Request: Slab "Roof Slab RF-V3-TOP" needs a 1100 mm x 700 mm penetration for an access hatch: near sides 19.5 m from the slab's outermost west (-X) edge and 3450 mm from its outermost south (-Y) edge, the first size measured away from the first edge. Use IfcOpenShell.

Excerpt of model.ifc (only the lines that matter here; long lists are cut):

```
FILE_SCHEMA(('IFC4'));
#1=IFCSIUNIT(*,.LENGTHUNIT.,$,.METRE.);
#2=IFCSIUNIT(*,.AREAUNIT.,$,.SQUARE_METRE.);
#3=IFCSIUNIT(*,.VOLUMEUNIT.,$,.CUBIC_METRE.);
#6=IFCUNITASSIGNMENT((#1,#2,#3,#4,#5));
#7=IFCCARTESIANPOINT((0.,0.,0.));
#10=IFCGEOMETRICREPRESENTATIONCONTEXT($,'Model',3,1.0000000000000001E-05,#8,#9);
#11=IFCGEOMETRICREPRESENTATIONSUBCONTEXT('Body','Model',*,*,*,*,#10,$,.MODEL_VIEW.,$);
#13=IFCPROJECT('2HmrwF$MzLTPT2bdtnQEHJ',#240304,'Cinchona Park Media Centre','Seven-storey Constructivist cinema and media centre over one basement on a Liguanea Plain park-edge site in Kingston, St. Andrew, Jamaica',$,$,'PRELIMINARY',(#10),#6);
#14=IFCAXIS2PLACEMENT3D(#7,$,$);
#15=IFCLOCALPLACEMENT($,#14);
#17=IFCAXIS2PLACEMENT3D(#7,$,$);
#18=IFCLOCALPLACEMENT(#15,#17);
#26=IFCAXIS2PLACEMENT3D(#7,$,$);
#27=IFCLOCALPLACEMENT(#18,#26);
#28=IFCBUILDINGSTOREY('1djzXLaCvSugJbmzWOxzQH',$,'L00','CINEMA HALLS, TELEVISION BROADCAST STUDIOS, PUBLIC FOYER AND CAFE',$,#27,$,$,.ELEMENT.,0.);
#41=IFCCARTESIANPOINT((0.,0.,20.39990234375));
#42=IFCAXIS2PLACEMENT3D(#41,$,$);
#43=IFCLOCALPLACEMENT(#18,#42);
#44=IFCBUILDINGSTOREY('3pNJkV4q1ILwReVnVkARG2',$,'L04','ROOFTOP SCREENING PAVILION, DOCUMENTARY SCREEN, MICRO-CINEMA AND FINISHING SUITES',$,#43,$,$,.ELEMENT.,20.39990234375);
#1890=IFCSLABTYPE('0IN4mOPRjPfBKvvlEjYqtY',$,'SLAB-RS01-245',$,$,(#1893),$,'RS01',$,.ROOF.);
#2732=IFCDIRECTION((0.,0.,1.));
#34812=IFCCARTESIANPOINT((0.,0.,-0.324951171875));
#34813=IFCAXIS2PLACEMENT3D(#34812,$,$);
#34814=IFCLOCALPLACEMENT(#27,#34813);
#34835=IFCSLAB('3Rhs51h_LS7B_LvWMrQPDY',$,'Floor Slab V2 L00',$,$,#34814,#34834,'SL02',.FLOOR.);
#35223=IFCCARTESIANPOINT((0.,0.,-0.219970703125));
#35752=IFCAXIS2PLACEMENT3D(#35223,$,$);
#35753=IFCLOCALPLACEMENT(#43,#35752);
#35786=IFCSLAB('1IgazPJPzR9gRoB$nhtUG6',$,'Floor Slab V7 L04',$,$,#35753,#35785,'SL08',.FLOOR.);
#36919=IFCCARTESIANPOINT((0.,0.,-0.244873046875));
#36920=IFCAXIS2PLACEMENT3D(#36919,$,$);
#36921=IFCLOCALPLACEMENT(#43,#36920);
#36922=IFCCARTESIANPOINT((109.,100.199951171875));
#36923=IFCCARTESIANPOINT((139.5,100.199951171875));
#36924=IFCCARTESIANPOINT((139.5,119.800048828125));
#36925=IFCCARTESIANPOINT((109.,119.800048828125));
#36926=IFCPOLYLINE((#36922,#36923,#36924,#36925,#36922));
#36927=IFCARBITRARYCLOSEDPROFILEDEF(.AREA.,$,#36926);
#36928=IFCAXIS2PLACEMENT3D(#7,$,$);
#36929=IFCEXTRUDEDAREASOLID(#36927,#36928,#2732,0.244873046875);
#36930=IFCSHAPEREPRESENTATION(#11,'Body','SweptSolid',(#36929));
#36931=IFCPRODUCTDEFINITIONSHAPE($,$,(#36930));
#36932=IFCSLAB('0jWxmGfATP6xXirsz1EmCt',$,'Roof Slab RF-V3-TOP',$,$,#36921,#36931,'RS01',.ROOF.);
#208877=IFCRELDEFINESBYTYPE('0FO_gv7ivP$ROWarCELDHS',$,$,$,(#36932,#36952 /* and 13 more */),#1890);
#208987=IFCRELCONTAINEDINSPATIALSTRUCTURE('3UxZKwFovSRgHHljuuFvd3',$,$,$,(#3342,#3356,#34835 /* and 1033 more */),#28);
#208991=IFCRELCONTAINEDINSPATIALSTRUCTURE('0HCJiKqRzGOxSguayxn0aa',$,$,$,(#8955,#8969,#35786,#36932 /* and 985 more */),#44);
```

```python
import numpy as np
import ifcopenshell
import ifcopenshell.api.feature
import ifcopenshell.api.geometry
import ifcopenshell.api.root
import ifcopenshell.geom
import ifcopenshell.util.placement
import ifcopenshell.util.representation
import ifcopenshell.util.shape
import ifcopenshell.util.unit

model = ifcopenshell.open("model.ifc")
unit_scale = ifcopenshell.util.unit.calculate_unit_scale(model)
settings = ifcopenshell.geom.settings()


def volume(element):
    """Net volume in cubic metres, openings subtracted."""
    shape = ifcopenshell.geom.create_shape(settings, element)
    return ifcopenshell.util.shape.get_volume(shape.geometry)


slab = model.by_guid("0jWxmGfATP6xXirsz1EmCt")
before = volume(slab)

# Extent in the slab's own axes, in metres. The edges named are its -X and -Y sides.
slab_shape = ifcopenshell.geom.create_shape(settings, slab)
vertices = ifcopenshell.util.shape.get_vertices(slab_shape.geometry)
x_min, y_min, bottom = vertices.min(axis=0)
top = vertices[:, 2].max()

opening = ifcopenshell.api.root.create_entity(model, ifc_class="IfcOpeningElement", name="Access hatch opening", predefined_type="OPENING")
context = ifcopenshell.util.representation.get_context(model, "Model", "Body", "MODEL_VIEW")
width, depth = 1.1, 0.7
outline = [(0.0, 0.0), (width, 0.0), (width, depth), (0.0, depth), (0.0, 0.0)]
# Overshoot both faces by 50 mm so the cut is clean.
shape = ifcopenshell.api.geometry.add_slab_representation(
    model, context=context, depth=top - bottom + 0.1, polyline=outline
)
ifcopenshell.api.geometry.assign_representation(model, product=opening, representation=shape)

matrix = ifcopenshell.util.placement.get_local_placement(slab.ObjectPlacement)
matrix[:, 3] = matrix @ np.append(np.array([x_min + 19.5, y_min + 3.45, bottom - 0.05]) / unit_scale, 1.0)
ifcopenshell.api.geometry.edit_object_placement(model, product=opening, matrix=matrix, is_si=False)
ifcopenshell.api.feature.add_feature(model, feature=opening, element=slab)

after = volume(slab)

print(f"slab volume {before:.3f} -> {after:.3f} m3")

model.write("model_edited.ifc")
```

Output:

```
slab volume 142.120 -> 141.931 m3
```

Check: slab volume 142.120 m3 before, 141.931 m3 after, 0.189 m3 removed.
